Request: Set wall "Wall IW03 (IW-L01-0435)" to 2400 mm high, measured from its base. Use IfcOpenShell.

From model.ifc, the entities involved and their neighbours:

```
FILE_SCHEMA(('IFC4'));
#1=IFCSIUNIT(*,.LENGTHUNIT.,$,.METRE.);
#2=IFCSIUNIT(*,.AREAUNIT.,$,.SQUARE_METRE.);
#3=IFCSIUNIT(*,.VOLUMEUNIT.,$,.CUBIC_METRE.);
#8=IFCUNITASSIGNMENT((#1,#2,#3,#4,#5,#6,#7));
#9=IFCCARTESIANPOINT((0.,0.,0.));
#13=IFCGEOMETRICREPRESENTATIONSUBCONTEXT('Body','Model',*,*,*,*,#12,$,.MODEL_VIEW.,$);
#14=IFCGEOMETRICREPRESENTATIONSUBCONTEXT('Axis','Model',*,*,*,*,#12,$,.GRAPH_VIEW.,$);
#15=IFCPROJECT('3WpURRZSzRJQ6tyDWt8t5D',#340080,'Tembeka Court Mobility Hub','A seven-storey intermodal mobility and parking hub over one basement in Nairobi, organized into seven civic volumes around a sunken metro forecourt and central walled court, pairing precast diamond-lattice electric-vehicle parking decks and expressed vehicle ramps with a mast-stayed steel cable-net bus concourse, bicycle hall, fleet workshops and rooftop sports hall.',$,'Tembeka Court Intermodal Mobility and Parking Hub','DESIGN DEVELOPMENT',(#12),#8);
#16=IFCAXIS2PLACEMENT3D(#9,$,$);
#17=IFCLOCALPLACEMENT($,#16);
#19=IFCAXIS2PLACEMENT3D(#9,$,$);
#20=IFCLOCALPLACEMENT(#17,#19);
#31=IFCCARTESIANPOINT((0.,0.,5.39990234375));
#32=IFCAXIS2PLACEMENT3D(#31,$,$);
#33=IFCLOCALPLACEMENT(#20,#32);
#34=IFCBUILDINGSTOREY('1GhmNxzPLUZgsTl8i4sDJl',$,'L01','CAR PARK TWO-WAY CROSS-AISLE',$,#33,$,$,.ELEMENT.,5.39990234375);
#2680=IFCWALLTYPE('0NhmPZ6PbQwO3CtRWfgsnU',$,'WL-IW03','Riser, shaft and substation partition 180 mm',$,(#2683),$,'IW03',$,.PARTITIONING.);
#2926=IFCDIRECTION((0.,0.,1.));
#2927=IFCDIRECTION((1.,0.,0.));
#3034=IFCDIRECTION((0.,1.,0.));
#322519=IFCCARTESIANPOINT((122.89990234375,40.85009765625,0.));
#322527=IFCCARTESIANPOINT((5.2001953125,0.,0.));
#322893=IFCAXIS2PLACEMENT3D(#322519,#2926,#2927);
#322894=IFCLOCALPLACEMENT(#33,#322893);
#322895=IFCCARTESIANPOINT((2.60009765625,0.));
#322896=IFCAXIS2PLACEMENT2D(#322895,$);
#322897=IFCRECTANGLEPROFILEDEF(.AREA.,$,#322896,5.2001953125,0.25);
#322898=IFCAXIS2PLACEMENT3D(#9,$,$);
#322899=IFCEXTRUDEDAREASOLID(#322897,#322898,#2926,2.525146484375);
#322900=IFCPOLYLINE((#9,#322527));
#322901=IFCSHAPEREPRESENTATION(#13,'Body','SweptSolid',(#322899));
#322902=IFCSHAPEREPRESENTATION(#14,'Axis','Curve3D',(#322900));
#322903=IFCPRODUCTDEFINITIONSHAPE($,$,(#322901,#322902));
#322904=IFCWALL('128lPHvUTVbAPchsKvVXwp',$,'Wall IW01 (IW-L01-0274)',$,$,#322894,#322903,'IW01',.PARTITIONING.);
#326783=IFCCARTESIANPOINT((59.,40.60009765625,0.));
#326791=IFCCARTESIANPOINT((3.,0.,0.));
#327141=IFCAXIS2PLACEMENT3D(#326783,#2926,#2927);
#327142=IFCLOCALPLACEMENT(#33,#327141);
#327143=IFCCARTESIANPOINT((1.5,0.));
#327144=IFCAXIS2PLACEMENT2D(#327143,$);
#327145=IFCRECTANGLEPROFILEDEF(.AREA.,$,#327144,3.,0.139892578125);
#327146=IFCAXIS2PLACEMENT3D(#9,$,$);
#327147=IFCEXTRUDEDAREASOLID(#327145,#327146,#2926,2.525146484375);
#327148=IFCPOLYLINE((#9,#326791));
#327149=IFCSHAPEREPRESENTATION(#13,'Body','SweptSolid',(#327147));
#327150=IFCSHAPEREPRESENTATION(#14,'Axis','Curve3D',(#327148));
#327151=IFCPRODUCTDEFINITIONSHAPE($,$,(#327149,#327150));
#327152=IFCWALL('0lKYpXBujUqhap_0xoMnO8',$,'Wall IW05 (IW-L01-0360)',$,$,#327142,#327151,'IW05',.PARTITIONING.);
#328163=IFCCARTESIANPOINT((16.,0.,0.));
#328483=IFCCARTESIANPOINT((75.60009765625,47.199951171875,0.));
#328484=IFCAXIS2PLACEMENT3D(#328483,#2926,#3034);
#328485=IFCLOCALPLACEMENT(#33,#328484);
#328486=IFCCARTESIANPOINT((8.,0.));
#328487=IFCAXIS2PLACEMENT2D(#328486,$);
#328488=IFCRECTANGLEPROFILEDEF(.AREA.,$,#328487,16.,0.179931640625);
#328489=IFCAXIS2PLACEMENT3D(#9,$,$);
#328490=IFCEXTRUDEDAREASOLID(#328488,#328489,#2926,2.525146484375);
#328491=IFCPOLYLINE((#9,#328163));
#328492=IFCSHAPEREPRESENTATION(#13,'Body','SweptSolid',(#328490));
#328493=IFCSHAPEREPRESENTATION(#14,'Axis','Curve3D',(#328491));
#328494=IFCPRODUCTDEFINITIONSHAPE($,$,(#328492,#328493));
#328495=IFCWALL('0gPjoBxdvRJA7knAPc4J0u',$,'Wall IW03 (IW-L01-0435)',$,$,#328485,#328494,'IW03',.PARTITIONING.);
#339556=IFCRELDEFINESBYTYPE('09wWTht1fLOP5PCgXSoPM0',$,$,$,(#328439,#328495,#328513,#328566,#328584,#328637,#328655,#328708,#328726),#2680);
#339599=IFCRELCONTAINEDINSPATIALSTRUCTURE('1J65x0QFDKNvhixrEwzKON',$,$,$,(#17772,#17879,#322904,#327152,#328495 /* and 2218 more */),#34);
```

```python
import ifcopenshell
import ifcopenshell.geom
import ifcopenshell.util.representation
import ifcopenshell.util.shape

model = ifcopenshell.open("model.ifc")
settings = ifcopenshell.geom.settings()


def volume(element):
    """Net volume in cubic metres, openings subtracted."""
    shape = ifcopenshell.geom.create_shape(settings, element)
    return ifcopenshell.util.shape.get_volume(shape.geometry)


wall = model.by_guid("0gPjoBxdvRJA7knAPc4J0u")
before = volume(wall)

body = ifcopenshell.util.representation.get_representation(wall, "Model", "Body")
solid = body.Items[0]
old_height = solid.Depth
solid.Depth = 2.4
after = volume(wall)

print(f"height {old_height:g} -> {solid.Depth:g}, volume {before:.3f} -> {after:.3f} m3")

model.write("model_v2.ifc")
```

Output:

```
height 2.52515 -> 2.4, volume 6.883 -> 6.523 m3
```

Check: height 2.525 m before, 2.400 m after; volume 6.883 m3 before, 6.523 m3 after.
